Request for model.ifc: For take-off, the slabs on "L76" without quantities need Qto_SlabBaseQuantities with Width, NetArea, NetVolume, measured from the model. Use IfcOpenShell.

First a look at what the model holds.

```python
import ifcopenshell
import ifcopenshell.util.element
import ifcopenshell.util.unit

model = ifcopenshell.open("model.ifc")
print(model.schema)
for unit_type in ("LENGTHUNIT", "AREAUNIT", "VOLUMEUNIT"):
    print(unit_type, ifcopenshell.util.unit.calculate_unit_scale(model, unit_type))
storey = next(s for s in model.by_type("IfcBuildingStorey") if s.Name == "L76")
slabs = [e for e in ifcopenshell.util.element.get_decomposition(storey) if e.is_a("IfcSlab")]
for e in sorted(slabs, key=lambda e: e.id()):
    print(e.id(), e.is_a(), e.Name, list(ifcopenshell.util.element.get_psets(e, qtos_only=True)), sep=" | ")
```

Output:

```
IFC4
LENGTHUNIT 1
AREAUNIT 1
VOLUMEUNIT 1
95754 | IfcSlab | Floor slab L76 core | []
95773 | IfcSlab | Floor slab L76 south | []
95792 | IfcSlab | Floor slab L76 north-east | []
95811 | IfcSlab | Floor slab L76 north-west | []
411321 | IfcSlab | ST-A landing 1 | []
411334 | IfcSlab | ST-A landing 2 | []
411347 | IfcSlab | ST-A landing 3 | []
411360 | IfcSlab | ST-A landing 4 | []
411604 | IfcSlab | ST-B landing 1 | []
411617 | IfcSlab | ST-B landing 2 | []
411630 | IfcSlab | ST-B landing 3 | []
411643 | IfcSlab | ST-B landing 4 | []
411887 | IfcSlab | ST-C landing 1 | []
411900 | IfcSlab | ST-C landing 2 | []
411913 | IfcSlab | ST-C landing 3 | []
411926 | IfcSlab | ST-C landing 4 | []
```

```python
import ifcopenshell
import ifcopenshell.api.pset
import ifcopenshell.geom
import ifcopenshell.util.element
import ifcopenshell.util.shape
import ifcopenshell.util.unit

model = ifcopenshell.open("model.ifc")
unit_scale = ifcopenshell.util.unit.calculate_unit_scale(model)
area_scale = ifcopenshell.util.unit.calculate_unit_scale(model, "AREAUNIT")
volume_scale = ifcopenshell.util.unit.calculate_unit_scale(model, "VOLUMEUNIT")
settings = ifcopenshell.geom.settings()

storey = next(s for s in model.by_type("IfcBuildingStorey") if s.Name == "L76")
slabs = [e for e in ifcopenshell.util.element.get_decomposition(storey) if e.is_a("IfcSlab")]

for e in sorted(slabs, key=lambda e: e.id()):
    if ifcopenshell.util.element.get_psets(e, qtos_only=True, should_inherit=False):
        continue
    # Geometry comes back in metres, in the element's own axes.
    shape = ifcopenshell.geom.create_shape(settings, e)
    values = {
        "Width": ifcopenshell.util.shape.get_z(shape.geometry) / unit_scale,
        "NetArea": ifcopenshell.util.shape.get_footprint_area(shape.geometry) / area_scale,
        "NetVolume": ifcopenshell.util.shape.get_volume(shape.geometry) / volume_scale,
    }
    qto = ifcopenshell.api.pset.add_qto(model, product=e, name="Qto_SlabBaseQuantities")
    ifcopenshell.api.pset.edit_qto(model, qto=qto, properties=values)
    print(e.id(), {k: round(v, 3) for k, v in values.items()})

model.write("model_rev.ifc")
```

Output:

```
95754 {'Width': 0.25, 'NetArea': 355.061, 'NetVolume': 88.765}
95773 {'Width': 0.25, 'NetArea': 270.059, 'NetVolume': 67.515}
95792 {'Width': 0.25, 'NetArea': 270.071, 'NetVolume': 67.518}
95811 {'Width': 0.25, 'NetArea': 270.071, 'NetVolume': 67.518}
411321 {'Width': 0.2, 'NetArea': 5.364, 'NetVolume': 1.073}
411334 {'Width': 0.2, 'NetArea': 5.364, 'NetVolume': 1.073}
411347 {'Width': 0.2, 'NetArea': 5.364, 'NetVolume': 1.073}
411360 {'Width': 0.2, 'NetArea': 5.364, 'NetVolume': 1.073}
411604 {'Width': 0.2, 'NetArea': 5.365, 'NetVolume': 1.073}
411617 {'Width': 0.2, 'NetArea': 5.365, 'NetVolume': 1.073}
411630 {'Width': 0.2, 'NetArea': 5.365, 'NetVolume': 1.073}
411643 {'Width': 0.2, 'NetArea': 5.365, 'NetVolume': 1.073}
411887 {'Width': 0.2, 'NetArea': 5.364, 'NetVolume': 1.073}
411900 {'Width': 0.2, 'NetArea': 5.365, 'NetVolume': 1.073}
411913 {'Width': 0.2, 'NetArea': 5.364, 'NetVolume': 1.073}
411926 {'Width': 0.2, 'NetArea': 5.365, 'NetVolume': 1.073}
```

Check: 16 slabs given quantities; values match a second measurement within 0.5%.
